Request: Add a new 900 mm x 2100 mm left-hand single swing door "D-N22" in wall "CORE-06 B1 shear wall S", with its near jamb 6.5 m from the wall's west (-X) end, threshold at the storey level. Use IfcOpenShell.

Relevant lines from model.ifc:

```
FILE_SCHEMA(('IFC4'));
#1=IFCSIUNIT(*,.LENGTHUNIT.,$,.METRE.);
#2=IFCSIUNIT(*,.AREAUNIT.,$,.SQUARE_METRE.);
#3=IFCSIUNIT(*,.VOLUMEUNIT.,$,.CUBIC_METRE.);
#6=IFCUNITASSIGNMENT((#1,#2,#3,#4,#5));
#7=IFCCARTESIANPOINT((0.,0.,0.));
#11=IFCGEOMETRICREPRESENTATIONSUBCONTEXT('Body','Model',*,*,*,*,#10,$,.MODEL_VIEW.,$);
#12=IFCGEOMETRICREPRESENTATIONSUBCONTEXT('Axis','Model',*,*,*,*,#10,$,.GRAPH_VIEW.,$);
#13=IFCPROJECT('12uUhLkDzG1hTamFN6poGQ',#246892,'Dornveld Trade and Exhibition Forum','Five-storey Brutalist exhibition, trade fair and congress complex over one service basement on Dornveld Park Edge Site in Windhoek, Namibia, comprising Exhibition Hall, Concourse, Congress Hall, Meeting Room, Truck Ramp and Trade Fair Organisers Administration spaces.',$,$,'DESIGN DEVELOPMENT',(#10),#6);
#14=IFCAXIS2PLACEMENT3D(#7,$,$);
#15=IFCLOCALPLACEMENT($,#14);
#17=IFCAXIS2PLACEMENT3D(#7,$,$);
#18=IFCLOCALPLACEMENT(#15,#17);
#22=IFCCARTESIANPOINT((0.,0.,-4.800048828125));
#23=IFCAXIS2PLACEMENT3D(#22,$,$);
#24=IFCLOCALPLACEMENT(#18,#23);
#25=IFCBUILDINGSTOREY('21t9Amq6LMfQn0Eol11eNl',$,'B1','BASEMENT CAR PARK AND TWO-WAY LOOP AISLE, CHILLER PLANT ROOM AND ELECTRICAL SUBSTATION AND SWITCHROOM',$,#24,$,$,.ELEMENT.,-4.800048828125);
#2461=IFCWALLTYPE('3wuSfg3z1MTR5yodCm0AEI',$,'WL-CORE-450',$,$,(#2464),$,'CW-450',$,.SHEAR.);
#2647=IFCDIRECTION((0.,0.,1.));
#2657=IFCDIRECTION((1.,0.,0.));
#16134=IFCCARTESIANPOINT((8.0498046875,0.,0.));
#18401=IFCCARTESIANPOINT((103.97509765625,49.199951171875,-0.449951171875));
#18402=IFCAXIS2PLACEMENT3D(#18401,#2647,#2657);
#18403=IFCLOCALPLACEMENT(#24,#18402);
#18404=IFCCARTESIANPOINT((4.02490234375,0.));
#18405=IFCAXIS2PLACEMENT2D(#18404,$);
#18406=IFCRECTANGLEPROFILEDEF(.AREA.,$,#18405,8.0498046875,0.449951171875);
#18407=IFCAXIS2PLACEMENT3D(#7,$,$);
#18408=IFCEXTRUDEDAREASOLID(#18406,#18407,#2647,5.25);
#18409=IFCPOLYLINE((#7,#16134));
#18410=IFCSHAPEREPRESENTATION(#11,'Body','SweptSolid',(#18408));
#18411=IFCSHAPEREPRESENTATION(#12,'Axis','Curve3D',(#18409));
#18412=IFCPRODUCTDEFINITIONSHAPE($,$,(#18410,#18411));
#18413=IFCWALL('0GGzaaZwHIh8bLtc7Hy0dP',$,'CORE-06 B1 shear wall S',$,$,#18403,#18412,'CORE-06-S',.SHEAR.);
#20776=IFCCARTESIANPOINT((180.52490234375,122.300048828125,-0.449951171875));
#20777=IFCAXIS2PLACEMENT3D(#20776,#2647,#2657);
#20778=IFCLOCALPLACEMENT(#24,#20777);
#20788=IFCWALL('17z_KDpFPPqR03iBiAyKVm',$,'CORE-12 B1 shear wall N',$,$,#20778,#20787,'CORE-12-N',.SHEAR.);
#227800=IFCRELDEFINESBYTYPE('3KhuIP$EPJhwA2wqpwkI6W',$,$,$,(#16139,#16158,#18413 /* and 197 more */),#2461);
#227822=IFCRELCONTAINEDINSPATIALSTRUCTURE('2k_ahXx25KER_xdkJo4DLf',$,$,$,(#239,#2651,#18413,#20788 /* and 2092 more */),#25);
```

```python
import numpy as np
import ifcopenshell
import ifcopenshell.api.feature
import ifcopenshell.api.geometry
import ifcopenshell.api.root
import ifcopenshell.api.spatial
import ifcopenshell.geom
import ifcopenshell.util.element
import ifcopenshell.util.placement
import ifcopenshell.util.representation
import ifcopenshell.util.shape
import ifcopenshell.util.unit

model = ifcopenshell.open("model.ifc")
unit_scale = ifcopenshell.util.unit.calculate_unit_scale(model)
settings = ifcopenshell.geom.settings()


def volume(element):
    """Net volume in cubic metres, openings subtracted."""
    shape = ifcopenshell.geom.create_shape(settings, element)
    return ifcopenshell.util.shape.get_volume(shape.geometry)


wall = model.by_guid("0GGzaaZwHIh8bLtc7Hy0dP")
storey = ifcopenshell.util.element.get_container(wall, ifc_class="IfcBuildingStorey")
context = ifcopenshell.util.representation.get_context(model, "Model", "Body", "MODEL_VIEW")
before = volume(wall)

width, height, from_end, sill = 0.9, 2.1, 6.5, 0.0  # metres

# The wall runs along its own X axis, and the end named is its -X end.
wall_shape = ifcopenshell.geom.create_shape(settings, wall)
x, y, z = ifcopenshell.util.shape.get_vertices(wall_shape.geometry).T
start = x.min() + from_end
face, thickness = float(y.min()), float(y.max() - y.min())
wall_matrix = ifcopenshell.util.placement.get_local_placement(wall.ObjectPlacement)
level = ifcopenshell.util.placement.get_local_placement(storey.ObjectPlacement)[2, 3]


def in_wall(x, y):
    """Placement at x, y metres in the wall's axes, at sill height."""
    matrix = wall_matrix.copy()
    matrix[:, 3] = wall_matrix @ np.array([x / unit_scale, y / unit_scale, 0.0, 1.0])
    matrix[2, 3] = level + sill / unit_scale
    return matrix


# Opening: a box that overshoots both wall faces by 50 mm.
opening = ifcopenshell.api.root.create_entity(model, ifc_class="IfcOpeningElement", predefined_type="OPENING")
box = ifcopenshell.api.geometry.add_wall_representation(
    model, context=context, length=width, height=height, thickness=thickness + 0.1
)
ifcopenshell.api.geometry.assign_representation(model, product=opening, representation=box)
ifcopenshell.api.geometry.edit_object_placement(model, product=opening, matrix=in_wall(start, face - 0.05), is_si=False)
ifcopenshell.api.feature.add_feature(model, feature=opening, element=wall)

door = ifcopenshell.api.root.create_entity(model, ifc_class="IfcDoor", name="D-N22", predefined_type="DOOR")
door.OverallWidth, door.OverallHeight = width / unit_scale, height / unit_scale
door.OperationType = "SINGLE_SWING_LEFT"
body = ifcopenshell.api.geometry.add_door_representation(
    model,
    context=context,
    overall_width=door.OverallWidth,
    overall_height=door.OverallHeight,
    operation_type="SINGLE_SWING_LEFT",
    lining_properties={"LiningDepth": thickness / unit_scale, "ThresholdDepth": thickness / unit_scale},
)
ifcopenshell.api.geometry.assign_representation(model, product=door, representation=body)
ifcopenshell.api.spatial.assign_container(model, products=[door], relating_structure=storey)
ifcopenshell.api.feature.add_filling(model, opening=opening, element=door)

# The lining spans the wall, so the door starts at the wall face.
ifcopenshell.api.geometry.edit_object_placement(model, product=door, matrix=in_wall(start, face), is_si=False)

after = volume(wall)

print(f"wall volume {before:.3f} -> {after:.3f} m3")

model.write("model_updated.ifc")
```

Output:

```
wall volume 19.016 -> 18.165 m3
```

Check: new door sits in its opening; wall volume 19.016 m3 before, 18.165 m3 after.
